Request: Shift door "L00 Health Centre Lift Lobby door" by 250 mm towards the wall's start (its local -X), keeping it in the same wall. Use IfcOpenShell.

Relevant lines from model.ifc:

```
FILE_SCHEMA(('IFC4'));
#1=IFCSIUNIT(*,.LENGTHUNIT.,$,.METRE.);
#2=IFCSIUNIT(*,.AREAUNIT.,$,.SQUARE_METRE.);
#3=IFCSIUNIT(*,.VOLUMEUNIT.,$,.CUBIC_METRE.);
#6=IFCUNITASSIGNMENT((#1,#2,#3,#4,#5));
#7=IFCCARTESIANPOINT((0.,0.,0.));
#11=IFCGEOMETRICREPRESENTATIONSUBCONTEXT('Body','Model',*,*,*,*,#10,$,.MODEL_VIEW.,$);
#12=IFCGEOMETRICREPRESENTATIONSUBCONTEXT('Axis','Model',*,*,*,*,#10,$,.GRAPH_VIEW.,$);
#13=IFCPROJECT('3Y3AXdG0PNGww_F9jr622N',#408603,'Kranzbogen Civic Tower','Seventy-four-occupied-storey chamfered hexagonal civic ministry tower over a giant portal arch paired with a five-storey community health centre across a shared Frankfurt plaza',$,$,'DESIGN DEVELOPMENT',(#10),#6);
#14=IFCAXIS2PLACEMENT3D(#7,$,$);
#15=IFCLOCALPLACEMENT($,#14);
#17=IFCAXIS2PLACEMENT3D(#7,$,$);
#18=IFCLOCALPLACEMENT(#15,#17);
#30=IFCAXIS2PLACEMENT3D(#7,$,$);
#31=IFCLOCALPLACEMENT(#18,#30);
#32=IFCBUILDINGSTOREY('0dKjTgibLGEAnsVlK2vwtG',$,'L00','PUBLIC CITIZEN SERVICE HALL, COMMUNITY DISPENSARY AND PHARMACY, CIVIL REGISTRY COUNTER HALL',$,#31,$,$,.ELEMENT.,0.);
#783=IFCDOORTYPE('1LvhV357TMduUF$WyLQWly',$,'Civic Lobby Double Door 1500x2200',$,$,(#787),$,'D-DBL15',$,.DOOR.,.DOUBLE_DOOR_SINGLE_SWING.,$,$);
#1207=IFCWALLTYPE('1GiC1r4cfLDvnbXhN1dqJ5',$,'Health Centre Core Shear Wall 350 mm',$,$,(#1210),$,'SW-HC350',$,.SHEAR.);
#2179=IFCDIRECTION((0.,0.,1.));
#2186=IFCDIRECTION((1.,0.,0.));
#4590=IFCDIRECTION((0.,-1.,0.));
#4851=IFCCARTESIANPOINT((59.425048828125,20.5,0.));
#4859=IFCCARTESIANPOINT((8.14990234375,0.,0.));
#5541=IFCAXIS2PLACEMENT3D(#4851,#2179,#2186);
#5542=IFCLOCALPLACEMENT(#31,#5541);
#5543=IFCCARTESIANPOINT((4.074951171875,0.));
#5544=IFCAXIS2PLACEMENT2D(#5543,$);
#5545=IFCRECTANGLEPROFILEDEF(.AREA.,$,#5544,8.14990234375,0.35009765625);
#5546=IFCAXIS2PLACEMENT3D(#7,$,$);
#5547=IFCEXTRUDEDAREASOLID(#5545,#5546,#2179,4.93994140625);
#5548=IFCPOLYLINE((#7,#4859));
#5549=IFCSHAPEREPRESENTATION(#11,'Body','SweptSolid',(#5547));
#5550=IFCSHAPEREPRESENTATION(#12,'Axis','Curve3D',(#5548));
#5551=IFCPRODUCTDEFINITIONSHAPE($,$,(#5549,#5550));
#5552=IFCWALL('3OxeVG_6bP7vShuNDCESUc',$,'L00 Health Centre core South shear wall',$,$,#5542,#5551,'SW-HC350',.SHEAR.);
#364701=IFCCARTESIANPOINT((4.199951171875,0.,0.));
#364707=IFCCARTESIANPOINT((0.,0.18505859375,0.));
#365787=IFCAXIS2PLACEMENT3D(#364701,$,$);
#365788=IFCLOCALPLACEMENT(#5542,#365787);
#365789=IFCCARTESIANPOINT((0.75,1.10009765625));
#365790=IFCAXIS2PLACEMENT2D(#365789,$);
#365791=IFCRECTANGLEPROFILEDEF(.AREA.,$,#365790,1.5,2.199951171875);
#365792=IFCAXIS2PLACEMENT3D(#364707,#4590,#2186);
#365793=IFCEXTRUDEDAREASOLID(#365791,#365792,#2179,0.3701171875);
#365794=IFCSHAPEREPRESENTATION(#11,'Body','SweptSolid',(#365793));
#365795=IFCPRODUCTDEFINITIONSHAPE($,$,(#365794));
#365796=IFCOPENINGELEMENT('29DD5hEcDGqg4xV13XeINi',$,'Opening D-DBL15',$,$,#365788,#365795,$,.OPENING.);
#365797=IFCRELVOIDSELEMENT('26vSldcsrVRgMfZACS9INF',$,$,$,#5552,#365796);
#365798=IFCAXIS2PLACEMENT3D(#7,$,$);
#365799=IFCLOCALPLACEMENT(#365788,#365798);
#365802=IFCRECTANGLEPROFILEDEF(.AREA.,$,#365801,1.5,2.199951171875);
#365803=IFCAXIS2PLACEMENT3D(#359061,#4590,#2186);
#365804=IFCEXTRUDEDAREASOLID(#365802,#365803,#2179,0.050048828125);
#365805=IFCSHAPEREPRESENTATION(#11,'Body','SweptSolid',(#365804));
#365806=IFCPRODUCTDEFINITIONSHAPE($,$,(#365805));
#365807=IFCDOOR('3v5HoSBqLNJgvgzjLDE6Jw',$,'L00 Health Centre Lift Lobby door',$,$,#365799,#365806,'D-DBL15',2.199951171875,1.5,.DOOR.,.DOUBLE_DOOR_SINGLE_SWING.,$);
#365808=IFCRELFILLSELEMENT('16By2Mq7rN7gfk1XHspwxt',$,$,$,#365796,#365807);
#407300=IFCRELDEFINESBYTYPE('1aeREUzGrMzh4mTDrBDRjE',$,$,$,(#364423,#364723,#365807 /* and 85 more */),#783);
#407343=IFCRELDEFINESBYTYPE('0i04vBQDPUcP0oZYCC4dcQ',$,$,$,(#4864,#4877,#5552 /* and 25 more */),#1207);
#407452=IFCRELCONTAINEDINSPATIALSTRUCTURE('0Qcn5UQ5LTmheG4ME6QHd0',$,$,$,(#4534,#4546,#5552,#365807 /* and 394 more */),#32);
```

```python
import ifcopenshell
import ifcopenshell.api.geometry
import ifcopenshell.util.placement
import ifcopenshell.util.unit

model = ifcopenshell.open("model.ifc")
unit_scale = ifcopenshell.util.unit.calculate_unit_scale(model)

door = model.by_id(365807)
opening = door.FillsVoids[0].RelatingOpeningElement
wall = opening.VoidsElements[0].RelatingBuildingElement

wall_matrix = ifcopenshell.util.placement.get_local_placement(wall.ObjectPlacement)
shift = wall_matrix[:3, 0] * -0.25 / unit_scale
before = ifcopenshell.util.placement.get_local_placement(door.ObjectPlacement)[:3, 3].copy()

# The door is placed relative to its opening, so it follows when the opening moves.
matrix = ifcopenshell.util.placement.get_local_placement(opening.ObjectPlacement)
matrix[:3, 3] += shift
ifcopenshell.api.geometry.edit_object_placement(
    model, product=opening, matrix=matrix, is_si=False, should_transform_children=True
)

after = ifcopenshell.util.placement.get_local_placement(door.ObjectPlacement)[:3, 3]
print("door moved by", (after - before).round(3) + 0.0)

model.write("model_v2.ifc")
```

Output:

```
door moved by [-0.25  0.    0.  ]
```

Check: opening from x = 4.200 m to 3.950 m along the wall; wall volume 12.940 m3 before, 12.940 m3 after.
